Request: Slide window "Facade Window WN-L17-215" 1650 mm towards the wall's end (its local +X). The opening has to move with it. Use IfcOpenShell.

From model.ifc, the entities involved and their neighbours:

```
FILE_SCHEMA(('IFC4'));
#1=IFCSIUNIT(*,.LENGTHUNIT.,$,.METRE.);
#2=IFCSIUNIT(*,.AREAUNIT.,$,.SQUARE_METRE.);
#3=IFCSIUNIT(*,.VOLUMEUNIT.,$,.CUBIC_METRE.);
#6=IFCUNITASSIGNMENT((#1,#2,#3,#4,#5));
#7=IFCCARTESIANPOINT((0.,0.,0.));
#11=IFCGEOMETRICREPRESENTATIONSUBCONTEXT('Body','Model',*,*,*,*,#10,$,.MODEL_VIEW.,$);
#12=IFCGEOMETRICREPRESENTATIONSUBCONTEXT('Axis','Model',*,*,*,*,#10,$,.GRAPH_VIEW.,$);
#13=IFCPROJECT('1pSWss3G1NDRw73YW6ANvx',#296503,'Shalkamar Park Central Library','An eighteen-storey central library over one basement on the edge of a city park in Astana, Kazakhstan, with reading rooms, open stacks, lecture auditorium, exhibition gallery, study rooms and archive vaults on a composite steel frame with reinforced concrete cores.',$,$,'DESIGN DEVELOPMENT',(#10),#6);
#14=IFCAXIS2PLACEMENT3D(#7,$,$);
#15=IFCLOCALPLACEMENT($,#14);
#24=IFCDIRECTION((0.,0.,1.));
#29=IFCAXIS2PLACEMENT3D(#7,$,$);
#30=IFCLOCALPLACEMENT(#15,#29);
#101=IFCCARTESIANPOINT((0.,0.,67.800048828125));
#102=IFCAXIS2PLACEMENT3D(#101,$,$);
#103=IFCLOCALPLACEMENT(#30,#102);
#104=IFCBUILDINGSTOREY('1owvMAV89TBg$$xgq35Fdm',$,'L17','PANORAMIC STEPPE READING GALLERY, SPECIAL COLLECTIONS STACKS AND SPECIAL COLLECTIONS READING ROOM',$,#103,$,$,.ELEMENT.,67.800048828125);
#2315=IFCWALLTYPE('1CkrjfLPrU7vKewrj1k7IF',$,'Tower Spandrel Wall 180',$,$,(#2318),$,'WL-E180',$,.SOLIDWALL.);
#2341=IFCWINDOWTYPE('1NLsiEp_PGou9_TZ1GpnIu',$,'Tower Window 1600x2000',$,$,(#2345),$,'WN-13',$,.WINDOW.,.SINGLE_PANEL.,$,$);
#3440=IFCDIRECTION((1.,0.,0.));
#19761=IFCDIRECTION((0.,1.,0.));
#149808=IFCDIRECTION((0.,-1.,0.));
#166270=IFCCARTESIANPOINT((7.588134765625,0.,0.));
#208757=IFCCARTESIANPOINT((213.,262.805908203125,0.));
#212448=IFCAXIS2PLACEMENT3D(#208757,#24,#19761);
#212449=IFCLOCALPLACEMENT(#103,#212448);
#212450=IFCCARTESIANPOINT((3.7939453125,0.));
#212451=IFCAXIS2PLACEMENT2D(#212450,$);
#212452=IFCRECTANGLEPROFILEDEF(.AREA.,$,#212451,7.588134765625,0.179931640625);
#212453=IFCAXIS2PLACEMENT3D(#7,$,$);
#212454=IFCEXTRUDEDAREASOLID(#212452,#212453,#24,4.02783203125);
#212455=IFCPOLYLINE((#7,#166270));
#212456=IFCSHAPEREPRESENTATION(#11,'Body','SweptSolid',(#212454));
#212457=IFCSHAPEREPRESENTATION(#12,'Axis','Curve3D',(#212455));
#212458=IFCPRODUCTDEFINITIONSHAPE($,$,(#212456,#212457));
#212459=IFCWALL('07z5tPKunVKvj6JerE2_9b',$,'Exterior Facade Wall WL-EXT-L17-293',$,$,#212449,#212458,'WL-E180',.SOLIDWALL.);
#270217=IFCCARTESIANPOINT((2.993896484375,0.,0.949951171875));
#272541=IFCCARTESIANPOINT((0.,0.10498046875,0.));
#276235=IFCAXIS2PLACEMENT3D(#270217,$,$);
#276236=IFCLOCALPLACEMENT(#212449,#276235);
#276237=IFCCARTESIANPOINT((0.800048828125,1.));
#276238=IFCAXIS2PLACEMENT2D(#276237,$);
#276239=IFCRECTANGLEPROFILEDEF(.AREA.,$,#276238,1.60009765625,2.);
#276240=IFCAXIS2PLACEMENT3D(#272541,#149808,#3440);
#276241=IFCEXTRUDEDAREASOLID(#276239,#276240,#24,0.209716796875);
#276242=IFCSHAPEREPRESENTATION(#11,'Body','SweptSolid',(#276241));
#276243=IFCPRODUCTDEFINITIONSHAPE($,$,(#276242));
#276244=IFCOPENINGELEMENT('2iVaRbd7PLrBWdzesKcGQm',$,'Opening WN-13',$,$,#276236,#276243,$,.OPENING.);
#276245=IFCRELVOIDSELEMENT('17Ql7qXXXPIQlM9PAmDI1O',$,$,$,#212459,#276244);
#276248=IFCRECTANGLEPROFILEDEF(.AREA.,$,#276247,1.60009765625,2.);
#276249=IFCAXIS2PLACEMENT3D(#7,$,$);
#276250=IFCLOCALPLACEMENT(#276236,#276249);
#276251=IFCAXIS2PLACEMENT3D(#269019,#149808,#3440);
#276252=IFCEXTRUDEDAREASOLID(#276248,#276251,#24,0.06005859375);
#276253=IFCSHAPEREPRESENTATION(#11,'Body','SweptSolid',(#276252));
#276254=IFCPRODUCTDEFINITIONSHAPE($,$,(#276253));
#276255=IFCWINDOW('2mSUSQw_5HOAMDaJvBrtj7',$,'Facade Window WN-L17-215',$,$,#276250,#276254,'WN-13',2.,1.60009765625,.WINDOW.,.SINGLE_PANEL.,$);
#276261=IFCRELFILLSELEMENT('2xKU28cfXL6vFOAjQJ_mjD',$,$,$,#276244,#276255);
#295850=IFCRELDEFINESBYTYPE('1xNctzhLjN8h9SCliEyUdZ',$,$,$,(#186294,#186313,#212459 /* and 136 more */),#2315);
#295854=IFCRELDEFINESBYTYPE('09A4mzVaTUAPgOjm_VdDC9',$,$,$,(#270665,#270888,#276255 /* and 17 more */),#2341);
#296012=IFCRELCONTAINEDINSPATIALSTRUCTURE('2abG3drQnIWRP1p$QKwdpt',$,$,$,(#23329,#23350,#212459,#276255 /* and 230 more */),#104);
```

```python
import ifcopenshell
import ifcopenshell.api.geometry
import ifcopenshell.util.placement
import ifcopenshell.util.unit

model = ifcopenshell.open("model.ifc")
unit_scale = ifcopenshell.util.unit.calculate_unit_scale(model)

window = model.by_guid("2mSUSQw_5HOAMDaJvBrtj7")
opening = window.FillsVoids[0].RelatingOpeningElement
wall = opening.VoidsElements[0].RelatingBuildingElement

wall_matrix = ifcopenshell.util.placement.get_local_placement(wall.ObjectPlacement)
shift = wall_matrix[:3, 0] * 1.65 / unit_scale
before = ifcopenshell.util.placement.get_local_placement(window.ObjectPlacement)[:3, 3].copy()

# The window is placed relative to its opening, so it follows when the opening moves.
matrix = ifcopenshell.util.placement.get_local_placement(opening.ObjectPlacement)
matrix[:3, 3] += shift
ifcopenshell.api.geometry.edit_object_placement(
    model, product=opening, matrix=matrix, is_si=False, should_transform_children=True
)

after = ifcopenshell.util.placement.get_local_placement(window.ObjectPlacement)[:3, 3]
print("window moved by", (after - before).round(3) + 0.0)

model.write("model_rev.ifc")
```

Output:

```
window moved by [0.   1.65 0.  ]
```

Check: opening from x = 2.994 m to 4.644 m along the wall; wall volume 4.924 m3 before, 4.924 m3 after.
